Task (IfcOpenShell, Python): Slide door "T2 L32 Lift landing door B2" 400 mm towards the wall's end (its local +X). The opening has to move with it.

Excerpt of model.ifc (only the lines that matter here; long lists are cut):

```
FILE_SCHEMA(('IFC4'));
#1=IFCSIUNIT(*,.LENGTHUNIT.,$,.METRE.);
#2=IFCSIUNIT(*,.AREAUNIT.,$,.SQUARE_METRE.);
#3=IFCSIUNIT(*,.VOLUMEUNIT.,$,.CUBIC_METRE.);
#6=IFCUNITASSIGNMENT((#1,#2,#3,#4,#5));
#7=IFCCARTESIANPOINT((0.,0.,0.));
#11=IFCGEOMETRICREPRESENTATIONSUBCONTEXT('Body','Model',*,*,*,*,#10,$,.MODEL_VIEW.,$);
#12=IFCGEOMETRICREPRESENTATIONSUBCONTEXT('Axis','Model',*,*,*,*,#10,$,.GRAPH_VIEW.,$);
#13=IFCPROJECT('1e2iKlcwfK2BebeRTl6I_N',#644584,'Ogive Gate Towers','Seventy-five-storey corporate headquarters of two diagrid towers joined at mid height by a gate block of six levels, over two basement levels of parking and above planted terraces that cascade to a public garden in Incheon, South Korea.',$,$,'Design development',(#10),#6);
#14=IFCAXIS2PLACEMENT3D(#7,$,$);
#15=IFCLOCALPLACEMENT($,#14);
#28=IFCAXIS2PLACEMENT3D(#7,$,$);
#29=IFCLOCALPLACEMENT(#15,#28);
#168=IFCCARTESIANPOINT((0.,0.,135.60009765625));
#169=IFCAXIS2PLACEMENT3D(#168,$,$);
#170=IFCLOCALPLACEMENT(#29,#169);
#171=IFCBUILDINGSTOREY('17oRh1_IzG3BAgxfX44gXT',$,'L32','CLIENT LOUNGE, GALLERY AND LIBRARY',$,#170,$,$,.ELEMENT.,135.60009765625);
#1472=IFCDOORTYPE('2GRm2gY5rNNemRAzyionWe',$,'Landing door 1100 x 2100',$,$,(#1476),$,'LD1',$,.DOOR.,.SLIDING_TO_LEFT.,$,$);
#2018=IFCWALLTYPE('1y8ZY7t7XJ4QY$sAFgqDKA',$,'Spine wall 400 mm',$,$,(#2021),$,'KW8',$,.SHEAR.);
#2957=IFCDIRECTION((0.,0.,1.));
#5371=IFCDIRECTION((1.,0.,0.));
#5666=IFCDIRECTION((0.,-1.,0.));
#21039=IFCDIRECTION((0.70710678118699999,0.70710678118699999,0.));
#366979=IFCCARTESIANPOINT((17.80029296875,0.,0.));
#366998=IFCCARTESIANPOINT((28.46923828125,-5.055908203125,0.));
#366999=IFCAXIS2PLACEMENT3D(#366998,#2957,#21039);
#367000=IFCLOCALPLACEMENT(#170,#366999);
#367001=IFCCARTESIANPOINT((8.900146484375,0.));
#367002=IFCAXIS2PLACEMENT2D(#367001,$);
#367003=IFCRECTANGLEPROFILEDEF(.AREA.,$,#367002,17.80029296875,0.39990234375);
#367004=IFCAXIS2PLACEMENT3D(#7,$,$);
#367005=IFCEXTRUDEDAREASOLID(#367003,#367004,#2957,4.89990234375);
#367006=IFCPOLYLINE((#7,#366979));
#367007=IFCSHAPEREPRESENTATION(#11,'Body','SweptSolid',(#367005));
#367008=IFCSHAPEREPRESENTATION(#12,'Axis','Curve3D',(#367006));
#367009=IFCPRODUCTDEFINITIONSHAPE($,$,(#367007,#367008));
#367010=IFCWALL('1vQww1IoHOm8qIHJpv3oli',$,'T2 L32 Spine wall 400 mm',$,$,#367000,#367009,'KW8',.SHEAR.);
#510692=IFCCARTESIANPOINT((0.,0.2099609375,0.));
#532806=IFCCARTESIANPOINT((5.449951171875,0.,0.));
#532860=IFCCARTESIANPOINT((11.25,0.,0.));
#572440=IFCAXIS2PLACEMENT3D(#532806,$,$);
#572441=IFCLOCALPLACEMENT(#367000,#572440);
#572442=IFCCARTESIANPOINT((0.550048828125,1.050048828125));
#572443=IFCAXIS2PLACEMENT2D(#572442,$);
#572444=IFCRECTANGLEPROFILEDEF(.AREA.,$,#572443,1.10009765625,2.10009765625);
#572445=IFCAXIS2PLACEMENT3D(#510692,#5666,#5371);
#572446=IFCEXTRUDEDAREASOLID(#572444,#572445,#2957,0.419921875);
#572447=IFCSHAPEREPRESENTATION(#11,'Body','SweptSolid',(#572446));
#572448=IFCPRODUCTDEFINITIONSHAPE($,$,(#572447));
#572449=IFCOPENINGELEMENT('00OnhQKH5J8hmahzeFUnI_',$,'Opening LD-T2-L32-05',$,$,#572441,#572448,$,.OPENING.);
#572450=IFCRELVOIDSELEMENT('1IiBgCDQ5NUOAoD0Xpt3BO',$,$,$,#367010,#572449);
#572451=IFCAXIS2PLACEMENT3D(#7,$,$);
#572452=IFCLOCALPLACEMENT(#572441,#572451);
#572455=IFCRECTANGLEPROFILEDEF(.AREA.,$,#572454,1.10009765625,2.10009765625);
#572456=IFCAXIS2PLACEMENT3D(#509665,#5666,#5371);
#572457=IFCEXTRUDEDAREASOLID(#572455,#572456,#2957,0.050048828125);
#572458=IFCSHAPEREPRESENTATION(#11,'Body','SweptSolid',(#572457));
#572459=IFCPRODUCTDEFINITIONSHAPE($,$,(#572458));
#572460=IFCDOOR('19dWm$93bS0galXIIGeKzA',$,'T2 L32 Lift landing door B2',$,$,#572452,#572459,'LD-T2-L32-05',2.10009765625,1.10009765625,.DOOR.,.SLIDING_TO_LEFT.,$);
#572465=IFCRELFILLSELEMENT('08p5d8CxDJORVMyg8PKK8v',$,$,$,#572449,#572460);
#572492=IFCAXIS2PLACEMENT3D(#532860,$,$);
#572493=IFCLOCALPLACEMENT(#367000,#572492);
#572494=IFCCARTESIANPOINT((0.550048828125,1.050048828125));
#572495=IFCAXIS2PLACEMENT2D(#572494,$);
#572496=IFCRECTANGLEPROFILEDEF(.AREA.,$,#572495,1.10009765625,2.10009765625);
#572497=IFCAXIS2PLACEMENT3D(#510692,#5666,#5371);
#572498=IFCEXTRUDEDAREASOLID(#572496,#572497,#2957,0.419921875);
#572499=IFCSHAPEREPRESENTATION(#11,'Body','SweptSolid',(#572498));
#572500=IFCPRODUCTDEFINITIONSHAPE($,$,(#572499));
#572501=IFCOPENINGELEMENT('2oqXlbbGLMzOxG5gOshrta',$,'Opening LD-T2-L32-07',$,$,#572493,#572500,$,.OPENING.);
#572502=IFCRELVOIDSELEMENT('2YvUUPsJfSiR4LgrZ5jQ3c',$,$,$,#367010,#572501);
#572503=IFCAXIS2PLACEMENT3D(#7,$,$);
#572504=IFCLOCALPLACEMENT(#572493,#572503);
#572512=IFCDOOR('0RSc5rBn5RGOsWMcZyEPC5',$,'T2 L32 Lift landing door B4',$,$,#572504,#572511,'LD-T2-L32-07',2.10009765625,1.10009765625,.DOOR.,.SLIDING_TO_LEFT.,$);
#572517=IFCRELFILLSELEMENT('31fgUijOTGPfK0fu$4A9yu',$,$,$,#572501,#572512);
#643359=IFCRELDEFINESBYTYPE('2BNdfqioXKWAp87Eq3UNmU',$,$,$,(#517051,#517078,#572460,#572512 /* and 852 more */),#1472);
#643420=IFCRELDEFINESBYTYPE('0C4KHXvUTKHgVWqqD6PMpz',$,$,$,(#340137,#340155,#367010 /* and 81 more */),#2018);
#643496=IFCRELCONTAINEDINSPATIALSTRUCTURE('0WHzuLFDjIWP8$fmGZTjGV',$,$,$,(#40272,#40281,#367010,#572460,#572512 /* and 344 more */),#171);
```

```python
import ifcopenshell
import ifcopenshell.api.geometry
import ifcopenshell.util.placement

model = ifcopenshell.open("model.ifc")

door = model.by_id(572460)
opening = door.FillsVoids[0].RelatingOpeningElement
wall = opening.VoidsElements[0].RelatingBuildingElement

wall_matrix = ifcopenshell.util.placement.get_local_placement(wall.ObjectPlacement)
shift = wall_matrix[:3, 0] * 0.4
before = ifcopenshell.util.placement.get_local_placement(door.ObjectPlacement)[:3, 3].copy()

# The door is placed relative to its opening, so it follows when the opening moves.
matrix = ifcopenshell.util.placement.get_local_placement(opening.ObjectPlacement)
matrix[:3, 3] += shift
ifcopenshell.api.geometry.edit_object_placement(
    model, product=opening, matrix=matrix, is_si=False, should_transform_children=True
)

after = ifcopenshell.util.placement.get_local_placement(door.ObjectPlacement)[:3, 3]
print("door moved by", (after - before).round(3) + 0.0)

model.write("model_edited.ifc")
```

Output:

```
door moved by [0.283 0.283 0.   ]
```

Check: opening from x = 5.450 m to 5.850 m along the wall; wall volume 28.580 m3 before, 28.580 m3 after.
